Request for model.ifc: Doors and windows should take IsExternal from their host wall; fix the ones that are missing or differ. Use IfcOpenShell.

First a look at what the model holds.

```python
import ifcopenshell
import ifcopenshell.util.element

model = ifcopenshell.open("model.ifc")
print(model.schema)
seen = {}
for e in model.by_type("IfcDoor") + model.by_type("IfcWindow"):
    if not e.FillsVoids:
        continue
    host = e.FillsVoids[0].RelatingOpeningElement.VoidsElements[0].RelatingBuildingElement
    own = ifcopenshell.util.element.get_pset(e, f"Pset_{e.is_a()[3:].removesuffix('StandardCase')}Common", "IsExternal")
    wall = ifcopenshell.util.element.get_pset(host, "Pset_WallCommon", "IsExternal")
    seen[e.is_a(), own, wall] = seen.get((e.is_a(), own, wall), 0) + 1
for (cls, own, wall), count in sorted(seen.items(), key=str):
    print(count, cls, "IsExternal:", own, "| host wall:", wall)
```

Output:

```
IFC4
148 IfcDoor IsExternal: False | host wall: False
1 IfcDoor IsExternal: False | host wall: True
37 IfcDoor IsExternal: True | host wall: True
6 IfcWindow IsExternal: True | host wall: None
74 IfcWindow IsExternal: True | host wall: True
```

```python
import ifcopenshell
import ifcopenshell.api.pset
import ifcopenshell.util.element

model = ifcopenshell.open("model.ifc")

count = 0
for ifc_class, pset_name in (("IfcDoor", "Pset_DoorCommon"), ("IfcWindow", "Pset_WindowCommon")):
    for e in model.by_type(ifc_class):
        if not e.FillsVoids:
            continue
        host = e.FillsVoids[0].RelatingOpeningElement.VoidsElements[0].RelatingBuildingElement
        external = ifcopenshell.util.element.get_pset(host, "Pset_WallCommon", "IsExternal")
        if external is None or ifcopenshell.util.element.get_pset(e, pset_name, "IsExternal") == external:
            continue
        pset = ifcopenshell.api.pset.add_pset(model, product=e, name=pset_name)
        ifcopenshell.api.pset.edit_pset(model, pset=pset, properties={"IsExternal": external})
        count += 1

print(count, "updated")

model.write("model_v2.ifc")
```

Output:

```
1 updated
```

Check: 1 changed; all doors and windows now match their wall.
